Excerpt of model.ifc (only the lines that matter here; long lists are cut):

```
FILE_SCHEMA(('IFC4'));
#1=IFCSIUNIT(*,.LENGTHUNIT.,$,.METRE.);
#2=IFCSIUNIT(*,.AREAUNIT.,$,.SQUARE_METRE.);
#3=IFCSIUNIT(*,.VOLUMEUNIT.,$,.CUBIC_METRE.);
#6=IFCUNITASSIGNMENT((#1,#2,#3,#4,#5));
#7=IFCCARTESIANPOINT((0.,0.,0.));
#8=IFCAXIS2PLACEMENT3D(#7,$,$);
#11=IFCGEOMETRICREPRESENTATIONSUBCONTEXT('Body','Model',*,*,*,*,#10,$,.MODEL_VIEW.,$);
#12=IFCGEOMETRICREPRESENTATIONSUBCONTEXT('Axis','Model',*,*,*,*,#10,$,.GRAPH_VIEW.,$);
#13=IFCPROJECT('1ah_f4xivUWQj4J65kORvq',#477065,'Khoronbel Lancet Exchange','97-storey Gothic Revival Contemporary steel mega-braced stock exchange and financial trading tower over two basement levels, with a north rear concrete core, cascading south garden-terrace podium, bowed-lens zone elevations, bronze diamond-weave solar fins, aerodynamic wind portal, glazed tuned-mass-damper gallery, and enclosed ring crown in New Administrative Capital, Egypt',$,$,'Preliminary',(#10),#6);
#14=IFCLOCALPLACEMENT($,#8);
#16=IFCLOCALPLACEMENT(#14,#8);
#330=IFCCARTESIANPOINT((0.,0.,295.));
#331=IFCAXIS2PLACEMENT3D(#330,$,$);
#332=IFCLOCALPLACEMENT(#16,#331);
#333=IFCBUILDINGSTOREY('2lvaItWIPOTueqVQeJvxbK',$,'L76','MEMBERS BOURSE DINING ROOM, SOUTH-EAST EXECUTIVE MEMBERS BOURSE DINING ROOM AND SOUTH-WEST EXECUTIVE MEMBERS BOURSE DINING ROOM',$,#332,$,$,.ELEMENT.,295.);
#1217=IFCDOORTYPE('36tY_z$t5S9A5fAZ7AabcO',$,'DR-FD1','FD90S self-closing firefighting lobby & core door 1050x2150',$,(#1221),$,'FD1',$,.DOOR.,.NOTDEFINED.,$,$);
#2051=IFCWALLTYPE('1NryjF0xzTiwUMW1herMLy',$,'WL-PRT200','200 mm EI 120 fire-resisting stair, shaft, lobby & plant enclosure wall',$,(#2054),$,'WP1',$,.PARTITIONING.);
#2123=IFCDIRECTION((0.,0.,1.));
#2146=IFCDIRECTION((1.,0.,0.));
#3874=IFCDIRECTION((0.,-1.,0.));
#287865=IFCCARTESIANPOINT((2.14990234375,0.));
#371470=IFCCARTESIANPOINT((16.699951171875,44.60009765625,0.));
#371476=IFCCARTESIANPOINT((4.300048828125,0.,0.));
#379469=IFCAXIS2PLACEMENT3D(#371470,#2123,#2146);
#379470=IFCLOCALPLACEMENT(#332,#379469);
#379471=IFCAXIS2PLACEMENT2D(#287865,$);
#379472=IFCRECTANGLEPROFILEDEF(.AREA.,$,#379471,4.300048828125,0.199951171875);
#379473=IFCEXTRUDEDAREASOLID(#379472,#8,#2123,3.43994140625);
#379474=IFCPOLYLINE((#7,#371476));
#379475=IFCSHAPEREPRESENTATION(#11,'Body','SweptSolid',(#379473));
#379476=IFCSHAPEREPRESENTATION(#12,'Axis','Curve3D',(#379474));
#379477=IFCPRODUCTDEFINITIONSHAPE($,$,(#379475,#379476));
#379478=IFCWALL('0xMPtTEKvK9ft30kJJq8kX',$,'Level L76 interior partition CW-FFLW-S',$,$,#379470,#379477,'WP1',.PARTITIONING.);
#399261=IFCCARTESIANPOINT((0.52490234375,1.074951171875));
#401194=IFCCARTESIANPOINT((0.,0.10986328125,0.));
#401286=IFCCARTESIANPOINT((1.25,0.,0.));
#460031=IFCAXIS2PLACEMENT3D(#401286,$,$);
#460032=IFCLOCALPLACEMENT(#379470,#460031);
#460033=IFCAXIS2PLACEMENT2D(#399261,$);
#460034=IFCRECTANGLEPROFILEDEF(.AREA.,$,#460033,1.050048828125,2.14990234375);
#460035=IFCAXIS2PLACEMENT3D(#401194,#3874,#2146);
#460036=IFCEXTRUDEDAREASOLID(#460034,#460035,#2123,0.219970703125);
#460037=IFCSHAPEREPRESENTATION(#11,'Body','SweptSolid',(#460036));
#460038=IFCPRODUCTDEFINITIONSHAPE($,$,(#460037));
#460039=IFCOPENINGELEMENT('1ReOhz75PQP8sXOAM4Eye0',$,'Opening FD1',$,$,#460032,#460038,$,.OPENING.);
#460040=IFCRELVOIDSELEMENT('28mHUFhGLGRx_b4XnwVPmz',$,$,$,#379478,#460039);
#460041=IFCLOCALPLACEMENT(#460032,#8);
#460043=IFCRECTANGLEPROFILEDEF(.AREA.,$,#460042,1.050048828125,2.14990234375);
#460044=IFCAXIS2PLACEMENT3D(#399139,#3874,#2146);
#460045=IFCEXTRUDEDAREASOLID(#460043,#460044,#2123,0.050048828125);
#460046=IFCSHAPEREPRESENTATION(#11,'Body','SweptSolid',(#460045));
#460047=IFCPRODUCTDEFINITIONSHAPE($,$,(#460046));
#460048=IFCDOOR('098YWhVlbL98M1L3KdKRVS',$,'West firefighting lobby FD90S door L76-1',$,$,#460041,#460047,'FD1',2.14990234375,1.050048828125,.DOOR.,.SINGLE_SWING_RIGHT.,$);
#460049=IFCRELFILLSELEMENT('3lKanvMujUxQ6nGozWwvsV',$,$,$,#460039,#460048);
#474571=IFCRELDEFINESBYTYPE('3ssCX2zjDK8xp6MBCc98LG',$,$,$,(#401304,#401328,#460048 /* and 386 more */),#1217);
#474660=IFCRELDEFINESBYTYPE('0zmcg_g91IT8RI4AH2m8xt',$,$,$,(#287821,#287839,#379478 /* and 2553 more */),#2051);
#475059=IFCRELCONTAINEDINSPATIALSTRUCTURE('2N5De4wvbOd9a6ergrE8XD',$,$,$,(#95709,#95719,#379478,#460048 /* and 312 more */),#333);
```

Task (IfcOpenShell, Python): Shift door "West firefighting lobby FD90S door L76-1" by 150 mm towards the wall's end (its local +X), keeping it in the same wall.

```python
import ifcopenshell
import ifcopenshell.api.geometry
import ifcopenshell.util.placement

model = ifcopenshell.open("model.ifc")

door = model.by_guid("098YWhVlbL98M1L3KdKRVS")
opening = door.FillsVoids[0].RelatingOpeningElement
wall = opening.VoidsElements[0].RelatingBuildingElement

wall_matrix = ifcopenshell.util.placement.get_local_placement(wall.ObjectPlacement)
shift = wall_matrix[:3, 0] * 0.15
before = ifcopenshell.util.placement.get_local_placement(door.ObjectPlacement)[:3, 3].copy()

# The door is placed relative to its opening, so it follows when the opening moves.
matrix = ifcopenshell.util.placement.get_local_placement(opening.ObjectPlacement)
matrix[:3, 3] += shift
ifcopenshell.api.geometry.edit_object_placement(
    model, product=opening, matrix=matrix, is_si=False, should_transform_children=True
)

after = ifcopenshell.util.placement.get_local_placement(door.ObjectPlacement)[:3, 3]
print("door moved by", (after - before).round(3) + 0.0)

model.write("model_rev.ifc")
```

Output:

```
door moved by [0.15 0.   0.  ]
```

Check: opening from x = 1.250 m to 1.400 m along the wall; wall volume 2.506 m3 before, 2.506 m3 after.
